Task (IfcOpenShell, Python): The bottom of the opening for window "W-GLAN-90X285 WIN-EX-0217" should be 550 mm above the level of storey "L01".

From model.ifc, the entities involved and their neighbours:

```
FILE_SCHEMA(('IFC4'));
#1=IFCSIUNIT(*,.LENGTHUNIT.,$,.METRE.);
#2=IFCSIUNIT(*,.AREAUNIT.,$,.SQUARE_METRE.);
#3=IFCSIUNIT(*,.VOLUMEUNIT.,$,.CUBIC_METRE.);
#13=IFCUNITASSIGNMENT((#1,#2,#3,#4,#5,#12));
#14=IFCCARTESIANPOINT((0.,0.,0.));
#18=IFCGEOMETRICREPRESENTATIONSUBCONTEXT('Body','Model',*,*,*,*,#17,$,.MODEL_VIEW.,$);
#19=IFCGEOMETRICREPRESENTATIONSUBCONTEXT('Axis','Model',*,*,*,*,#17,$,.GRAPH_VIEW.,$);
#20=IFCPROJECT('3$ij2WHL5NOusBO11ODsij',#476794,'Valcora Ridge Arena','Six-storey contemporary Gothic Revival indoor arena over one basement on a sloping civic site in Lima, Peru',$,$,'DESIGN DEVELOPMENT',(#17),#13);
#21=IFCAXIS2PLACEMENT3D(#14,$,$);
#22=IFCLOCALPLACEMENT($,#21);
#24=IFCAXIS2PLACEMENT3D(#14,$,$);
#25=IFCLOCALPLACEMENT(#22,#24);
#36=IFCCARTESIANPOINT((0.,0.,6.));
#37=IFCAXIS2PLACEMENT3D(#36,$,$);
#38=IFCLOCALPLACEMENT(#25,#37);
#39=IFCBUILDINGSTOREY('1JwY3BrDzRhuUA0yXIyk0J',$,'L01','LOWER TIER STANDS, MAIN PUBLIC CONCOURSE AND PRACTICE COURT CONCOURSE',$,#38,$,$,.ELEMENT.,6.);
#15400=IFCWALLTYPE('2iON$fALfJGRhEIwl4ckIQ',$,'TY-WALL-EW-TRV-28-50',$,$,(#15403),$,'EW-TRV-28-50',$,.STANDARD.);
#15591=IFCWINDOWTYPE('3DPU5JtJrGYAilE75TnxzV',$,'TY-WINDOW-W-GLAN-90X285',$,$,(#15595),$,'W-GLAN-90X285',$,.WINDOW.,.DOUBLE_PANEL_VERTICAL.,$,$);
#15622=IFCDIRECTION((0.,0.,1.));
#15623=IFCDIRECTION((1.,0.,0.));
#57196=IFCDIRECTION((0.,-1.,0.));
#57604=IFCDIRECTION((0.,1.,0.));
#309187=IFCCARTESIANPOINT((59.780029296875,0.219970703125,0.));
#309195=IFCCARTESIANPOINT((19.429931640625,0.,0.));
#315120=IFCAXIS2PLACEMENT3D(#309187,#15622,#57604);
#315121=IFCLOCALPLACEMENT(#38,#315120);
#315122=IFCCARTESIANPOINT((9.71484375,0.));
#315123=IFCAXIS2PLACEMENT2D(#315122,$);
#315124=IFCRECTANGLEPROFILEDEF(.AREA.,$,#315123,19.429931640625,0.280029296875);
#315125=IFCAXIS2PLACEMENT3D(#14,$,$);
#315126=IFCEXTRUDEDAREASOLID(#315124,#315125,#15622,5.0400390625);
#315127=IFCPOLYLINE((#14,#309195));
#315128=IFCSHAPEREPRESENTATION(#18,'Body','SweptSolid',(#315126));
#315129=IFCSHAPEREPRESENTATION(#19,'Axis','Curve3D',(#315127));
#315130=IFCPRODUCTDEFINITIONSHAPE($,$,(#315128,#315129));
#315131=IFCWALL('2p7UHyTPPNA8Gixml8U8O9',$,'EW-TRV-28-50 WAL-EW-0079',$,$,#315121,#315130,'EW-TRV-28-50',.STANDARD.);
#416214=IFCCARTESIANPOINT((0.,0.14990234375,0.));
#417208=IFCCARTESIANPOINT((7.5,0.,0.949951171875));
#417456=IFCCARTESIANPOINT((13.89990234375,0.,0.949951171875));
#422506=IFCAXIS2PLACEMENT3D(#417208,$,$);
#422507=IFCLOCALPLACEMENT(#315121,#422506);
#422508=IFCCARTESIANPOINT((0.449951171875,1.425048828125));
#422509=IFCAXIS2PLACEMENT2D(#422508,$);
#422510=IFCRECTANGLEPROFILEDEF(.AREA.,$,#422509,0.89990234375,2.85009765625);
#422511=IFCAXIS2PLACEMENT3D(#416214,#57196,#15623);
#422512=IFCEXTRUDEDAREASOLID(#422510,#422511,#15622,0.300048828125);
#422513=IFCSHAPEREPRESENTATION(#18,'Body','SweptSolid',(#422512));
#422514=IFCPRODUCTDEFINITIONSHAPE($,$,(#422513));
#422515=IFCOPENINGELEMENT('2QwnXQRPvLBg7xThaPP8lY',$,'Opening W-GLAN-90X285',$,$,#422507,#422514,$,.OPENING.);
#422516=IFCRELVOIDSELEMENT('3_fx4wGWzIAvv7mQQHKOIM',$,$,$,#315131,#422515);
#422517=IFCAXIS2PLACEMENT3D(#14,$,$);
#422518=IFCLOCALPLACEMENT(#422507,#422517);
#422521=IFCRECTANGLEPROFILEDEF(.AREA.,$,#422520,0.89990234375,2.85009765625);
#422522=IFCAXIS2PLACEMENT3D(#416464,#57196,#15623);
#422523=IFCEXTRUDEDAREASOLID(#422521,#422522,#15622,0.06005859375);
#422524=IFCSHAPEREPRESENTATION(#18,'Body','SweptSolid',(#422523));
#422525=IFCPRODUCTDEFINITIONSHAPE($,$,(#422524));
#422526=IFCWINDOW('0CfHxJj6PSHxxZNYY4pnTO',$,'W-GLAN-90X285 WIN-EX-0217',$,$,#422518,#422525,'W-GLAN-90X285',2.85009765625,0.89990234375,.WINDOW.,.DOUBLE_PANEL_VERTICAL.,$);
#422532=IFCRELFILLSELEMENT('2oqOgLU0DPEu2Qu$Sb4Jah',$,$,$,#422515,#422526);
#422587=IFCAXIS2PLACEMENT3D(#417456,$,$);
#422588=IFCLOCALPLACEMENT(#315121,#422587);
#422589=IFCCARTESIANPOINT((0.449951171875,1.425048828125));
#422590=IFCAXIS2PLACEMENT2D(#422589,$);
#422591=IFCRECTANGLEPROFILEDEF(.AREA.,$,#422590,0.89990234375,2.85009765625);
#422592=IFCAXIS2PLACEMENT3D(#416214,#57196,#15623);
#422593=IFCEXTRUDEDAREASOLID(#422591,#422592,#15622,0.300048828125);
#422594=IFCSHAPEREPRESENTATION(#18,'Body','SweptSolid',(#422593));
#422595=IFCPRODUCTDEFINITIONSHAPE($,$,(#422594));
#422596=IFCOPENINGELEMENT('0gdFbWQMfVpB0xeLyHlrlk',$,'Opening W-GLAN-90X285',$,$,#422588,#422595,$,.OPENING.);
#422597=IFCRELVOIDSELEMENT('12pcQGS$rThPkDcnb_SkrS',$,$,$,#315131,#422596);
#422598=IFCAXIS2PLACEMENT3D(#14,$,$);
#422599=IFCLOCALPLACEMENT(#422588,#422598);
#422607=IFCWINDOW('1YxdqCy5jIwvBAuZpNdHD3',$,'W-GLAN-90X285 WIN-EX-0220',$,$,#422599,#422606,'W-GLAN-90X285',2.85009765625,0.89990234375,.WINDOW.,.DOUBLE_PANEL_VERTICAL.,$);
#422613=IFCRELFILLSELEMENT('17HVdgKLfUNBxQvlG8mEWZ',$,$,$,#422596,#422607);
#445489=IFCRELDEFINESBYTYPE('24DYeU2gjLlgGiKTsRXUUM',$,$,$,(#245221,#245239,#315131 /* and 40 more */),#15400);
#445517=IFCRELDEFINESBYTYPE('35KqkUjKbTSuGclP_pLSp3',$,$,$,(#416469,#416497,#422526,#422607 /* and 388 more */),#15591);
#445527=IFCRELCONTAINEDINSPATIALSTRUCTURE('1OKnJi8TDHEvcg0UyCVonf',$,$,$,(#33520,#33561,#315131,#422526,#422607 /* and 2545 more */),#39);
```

```python
import numpy as np
import ifcopenshell
import ifcopenshell.api.geometry
import ifcopenshell.geom
import ifcopenshell.util.element
import ifcopenshell.util.placement
import ifcopenshell.util.shape
import ifcopenshell.util.unit

model = ifcopenshell.open("model.ifc")
unit_scale = ifcopenshell.util.unit.calculate_unit_scale(model)

window = model.by_guid("0CfHxJj6PSHxxZNYY4pnTO")
opening = window.FillsVoids[0].RelatingOpeningElement
storey = ifcopenshell.util.element.get_container(window, ifc_class="IfcBuildingStorey")
level = ifcopenshell.util.placement.get_local_placement(storey.ObjectPlacement)[2, 3]

# The opening's origin need not be at the sill, so measure its lowest point.
shape = ifcopenshell.geom.create_shape(ifcopenshell.geom.settings(), opening)
bottom = ifcopenshell.util.shape.get_shape_bottom_elevation(shape, shape.geometry) / unit_scale
dz = level + 0.55 / unit_scale - bottom

shift = np.array([0.0, 0.0, dz])
# The window is placed relative to its opening, so it follows when the opening moves.
matrix = ifcopenshell.util.placement.get_local_placement(opening.ObjectPlacement)
matrix[:3, 3] += shift
ifcopenshell.api.geometry.edit_object_placement(
    model, product=opening, matrix=matrix, is_si=False, should_transform_children=True
)

print(f"moved by {dz * unit_scale:+.3f} m")

model.write("model_rev.ifc")
```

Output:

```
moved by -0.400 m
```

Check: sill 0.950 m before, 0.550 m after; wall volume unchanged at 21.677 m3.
